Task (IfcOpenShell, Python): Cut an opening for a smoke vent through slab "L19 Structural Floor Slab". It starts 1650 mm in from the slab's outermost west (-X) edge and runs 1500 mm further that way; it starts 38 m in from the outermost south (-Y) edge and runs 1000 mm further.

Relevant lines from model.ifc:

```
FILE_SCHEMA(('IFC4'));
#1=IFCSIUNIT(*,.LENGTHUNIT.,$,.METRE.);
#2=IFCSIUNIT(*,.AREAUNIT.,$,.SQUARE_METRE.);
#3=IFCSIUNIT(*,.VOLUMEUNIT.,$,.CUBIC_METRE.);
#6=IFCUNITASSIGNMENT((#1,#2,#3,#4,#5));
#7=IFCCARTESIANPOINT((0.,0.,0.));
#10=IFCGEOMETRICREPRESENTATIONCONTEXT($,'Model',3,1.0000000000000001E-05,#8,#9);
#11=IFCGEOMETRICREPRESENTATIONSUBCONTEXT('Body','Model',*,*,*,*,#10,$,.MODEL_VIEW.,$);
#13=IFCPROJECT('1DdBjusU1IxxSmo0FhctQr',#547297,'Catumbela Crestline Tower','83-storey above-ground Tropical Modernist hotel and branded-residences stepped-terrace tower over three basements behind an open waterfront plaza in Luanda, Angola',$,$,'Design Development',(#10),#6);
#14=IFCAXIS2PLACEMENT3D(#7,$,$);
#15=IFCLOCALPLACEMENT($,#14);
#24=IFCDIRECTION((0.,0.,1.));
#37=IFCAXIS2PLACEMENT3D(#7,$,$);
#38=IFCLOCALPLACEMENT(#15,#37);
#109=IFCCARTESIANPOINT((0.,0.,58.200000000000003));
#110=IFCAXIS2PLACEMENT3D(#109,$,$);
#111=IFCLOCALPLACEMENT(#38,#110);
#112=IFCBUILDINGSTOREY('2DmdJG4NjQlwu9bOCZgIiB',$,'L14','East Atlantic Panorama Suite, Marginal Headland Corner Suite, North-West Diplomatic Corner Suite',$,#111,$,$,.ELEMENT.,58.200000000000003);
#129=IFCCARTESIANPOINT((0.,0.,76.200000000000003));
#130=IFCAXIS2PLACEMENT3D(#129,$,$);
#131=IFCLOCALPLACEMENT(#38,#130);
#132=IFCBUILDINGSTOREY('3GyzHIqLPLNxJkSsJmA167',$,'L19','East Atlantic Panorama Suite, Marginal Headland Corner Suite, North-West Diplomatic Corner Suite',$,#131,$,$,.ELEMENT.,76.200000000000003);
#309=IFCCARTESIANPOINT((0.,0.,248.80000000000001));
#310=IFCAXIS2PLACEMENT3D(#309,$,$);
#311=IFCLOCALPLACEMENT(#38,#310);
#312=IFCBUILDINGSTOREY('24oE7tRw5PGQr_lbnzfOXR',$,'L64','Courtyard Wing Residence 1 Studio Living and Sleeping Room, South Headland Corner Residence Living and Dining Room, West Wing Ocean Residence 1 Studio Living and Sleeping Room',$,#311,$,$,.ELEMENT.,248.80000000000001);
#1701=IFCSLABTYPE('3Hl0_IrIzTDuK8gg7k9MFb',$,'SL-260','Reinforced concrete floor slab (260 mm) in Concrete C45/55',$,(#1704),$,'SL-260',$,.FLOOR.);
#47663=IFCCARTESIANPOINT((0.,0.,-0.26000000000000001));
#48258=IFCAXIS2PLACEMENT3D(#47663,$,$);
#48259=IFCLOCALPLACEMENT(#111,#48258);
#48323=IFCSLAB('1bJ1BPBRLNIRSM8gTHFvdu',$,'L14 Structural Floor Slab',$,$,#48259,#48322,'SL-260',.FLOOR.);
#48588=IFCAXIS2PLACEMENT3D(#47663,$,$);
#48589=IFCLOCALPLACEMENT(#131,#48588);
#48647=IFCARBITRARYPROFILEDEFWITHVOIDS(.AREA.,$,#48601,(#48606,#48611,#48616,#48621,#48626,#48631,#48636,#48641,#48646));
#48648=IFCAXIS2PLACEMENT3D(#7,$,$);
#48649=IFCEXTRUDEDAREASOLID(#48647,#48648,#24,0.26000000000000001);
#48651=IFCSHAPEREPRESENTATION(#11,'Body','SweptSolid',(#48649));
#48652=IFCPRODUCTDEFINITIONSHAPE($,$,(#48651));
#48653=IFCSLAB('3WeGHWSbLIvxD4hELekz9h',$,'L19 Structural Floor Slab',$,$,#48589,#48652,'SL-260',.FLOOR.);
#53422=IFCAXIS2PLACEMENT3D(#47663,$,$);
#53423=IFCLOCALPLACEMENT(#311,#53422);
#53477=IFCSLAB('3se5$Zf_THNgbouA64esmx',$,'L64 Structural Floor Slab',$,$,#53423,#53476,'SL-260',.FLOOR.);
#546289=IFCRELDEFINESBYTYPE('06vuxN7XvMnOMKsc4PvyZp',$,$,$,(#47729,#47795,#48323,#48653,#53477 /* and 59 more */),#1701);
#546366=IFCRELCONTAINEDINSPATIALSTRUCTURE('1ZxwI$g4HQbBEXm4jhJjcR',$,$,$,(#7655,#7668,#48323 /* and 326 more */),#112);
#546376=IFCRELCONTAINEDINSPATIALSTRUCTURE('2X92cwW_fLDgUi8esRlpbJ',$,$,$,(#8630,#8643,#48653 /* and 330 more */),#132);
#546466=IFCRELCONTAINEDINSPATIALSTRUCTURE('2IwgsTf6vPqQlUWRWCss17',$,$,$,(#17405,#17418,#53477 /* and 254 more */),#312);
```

```python
import numpy as np
import ifcopenshell
import ifcopenshell.api.feature
import ifcopenshell.api.geometry
import ifcopenshell.api.root
import ifcopenshell.geom
import ifcopenshell.util.placement
import ifcopenshell.util.representation
import ifcopenshell.util.shape
import ifcopenshell.util.unit

model = ifcopenshell.open("model.ifc")
unit_scale = ifcopenshell.util.unit.calculate_unit_scale(model)
settings = ifcopenshell.geom.settings()


def volume(element):
    """Net volume in cubic metres, openings subtracted."""
    shape = ifcopenshell.geom.create_shape(settings, element)
    return ifcopenshell.util.shape.get_volume(shape.geometry)


slab = model.by_guid("3WeGHWSbLIvxD4hELekz9h")
before = volume(slab)

# Extent in the slab's own axes, in metres. The edges named are its -X and -Y sides.
slab_shape = ifcopenshell.geom.create_shape(settings, slab)
vertices = ifcopenshell.util.shape.get_vertices(slab_shape.geometry)
x_min, y_min, bottom = vertices.min(axis=0)
top = vertices[:, 2].max()

opening = ifcopenshell.api.root.create_entity(model, ifc_class="IfcOpeningElement", name="Smoke vent opening", predefined_type="OPENING")
context = ifcopenshell.util.representation.get_context(model, "Model", "Body", "MODEL_VIEW")
width, depth = 1.5, 1
outline = [(0.0, 0.0), (width, 0.0), (width, depth), (0.0, depth), (0.0, 0.0)]
# Overshoot both faces by 50 mm so the cut is clean.
shape = ifcopenshell.api.geometry.add_slab_representation(
    model, context=context, depth=top - bottom + 0.1, polyline=outline
)
ifcopenshell.api.geometry.assign_representation(model, product=opening, representation=shape)

matrix = ifcopenshell.util.placement.get_local_placement(slab.ObjectPlacement)
matrix[:, 3] = matrix @ np.append(np.array([x_min + 1.65, y_min + 38, bottom - 0.05]) / unit_scale, 1.0)
ifcopenshell.api.geometry.edit_object_placement(model, product=opening, matrix=matrix, is_si=False)
ifcopenshell.api.feature.add_feature(model, feature=opening, element=slab)

after = volume(slab)

print(f"slab volume {before:.3f} -> {after:.3f} m3")

model.write("model-out.ifc")
```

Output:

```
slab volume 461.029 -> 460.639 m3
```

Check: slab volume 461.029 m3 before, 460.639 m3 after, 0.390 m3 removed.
